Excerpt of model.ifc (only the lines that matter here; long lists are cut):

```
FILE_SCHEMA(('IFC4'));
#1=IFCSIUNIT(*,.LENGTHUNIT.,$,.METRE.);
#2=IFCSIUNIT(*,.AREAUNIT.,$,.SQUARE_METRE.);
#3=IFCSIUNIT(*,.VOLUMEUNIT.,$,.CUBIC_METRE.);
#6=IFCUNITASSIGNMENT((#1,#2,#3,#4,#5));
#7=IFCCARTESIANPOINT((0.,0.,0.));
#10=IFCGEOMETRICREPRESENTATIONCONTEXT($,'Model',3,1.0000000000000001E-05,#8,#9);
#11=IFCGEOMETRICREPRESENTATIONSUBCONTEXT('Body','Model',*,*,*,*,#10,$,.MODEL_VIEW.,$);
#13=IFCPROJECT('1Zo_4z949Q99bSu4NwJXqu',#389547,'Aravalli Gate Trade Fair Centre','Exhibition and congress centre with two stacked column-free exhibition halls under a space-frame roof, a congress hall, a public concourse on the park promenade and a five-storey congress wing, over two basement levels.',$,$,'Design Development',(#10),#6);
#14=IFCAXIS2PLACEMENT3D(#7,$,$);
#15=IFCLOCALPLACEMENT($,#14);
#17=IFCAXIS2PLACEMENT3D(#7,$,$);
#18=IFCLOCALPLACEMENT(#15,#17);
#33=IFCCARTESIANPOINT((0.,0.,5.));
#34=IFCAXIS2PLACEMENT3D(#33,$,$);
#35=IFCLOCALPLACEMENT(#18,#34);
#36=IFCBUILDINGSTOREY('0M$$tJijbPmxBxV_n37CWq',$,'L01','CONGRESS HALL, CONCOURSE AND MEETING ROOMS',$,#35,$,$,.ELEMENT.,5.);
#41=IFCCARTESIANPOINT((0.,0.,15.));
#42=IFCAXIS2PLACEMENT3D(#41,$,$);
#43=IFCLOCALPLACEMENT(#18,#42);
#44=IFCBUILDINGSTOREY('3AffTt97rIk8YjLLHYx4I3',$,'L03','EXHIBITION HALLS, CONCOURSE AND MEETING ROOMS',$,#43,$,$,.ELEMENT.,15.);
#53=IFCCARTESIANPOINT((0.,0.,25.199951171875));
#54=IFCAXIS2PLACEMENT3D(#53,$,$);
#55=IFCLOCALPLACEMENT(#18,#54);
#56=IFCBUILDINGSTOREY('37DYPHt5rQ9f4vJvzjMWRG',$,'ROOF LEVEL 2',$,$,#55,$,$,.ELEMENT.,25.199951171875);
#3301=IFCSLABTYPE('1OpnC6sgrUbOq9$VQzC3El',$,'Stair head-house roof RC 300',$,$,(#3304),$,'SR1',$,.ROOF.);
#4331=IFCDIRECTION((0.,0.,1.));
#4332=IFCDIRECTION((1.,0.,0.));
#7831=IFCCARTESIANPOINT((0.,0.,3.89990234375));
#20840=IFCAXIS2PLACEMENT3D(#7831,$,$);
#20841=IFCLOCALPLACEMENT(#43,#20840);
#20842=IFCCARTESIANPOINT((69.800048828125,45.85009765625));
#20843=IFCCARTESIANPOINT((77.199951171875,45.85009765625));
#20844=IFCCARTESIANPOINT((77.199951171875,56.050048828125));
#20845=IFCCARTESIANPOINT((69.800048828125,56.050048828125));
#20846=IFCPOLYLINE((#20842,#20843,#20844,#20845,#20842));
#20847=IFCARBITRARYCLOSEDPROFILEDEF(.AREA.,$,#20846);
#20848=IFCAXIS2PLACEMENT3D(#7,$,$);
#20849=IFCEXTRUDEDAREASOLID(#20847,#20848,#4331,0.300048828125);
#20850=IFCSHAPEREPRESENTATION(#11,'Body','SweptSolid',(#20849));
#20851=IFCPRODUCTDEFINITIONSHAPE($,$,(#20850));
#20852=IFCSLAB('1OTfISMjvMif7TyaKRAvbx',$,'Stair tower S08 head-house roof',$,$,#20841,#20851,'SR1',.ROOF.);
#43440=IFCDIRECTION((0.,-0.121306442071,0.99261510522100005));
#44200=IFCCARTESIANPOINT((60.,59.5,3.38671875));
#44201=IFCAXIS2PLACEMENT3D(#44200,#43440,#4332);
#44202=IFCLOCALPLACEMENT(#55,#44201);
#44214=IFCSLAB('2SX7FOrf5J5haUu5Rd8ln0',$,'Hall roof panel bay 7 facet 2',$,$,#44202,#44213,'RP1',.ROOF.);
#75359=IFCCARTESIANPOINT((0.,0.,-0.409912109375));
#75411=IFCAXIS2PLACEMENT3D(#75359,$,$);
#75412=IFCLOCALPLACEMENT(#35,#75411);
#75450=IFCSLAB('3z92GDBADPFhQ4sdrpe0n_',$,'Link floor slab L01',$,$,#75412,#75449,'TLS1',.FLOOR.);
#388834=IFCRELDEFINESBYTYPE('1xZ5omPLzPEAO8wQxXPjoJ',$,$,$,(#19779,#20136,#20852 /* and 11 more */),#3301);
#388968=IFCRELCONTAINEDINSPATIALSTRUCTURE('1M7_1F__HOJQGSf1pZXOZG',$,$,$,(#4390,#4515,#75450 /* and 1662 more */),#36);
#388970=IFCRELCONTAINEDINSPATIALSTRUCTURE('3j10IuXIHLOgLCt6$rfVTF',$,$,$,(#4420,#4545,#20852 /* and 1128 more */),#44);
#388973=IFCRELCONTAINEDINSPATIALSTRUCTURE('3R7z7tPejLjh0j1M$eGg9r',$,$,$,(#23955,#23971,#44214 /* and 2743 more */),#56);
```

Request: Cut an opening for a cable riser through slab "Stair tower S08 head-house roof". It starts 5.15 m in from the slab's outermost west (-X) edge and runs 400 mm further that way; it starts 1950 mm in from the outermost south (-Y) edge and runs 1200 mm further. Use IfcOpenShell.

```python
import numpy as np
import ifcopenshell
import ifcopenshell.api.feature
import ifcopenshell.api.geometry
import ifcopenshell.api.root
import ifcopenshell.geom
import ifcopenshell.util.placement
import ifcopenshell.util.representation
import ifcopenshell.util.shape
import ifcopenshell.util.unit

model = ifcopenshell.open("model.ifc")
unit_scale = ifcopenshell.util.unit.calculate_unit_scale(model)
settings = ifcopenshell.geom.settings()


def volume(element):
    """Net volume in cubic metres, openings subtracted."""
    shape = ifcopenshell.geom.create_shape(settings, element)
    return ifcopenshell.util.shape.get_volume(shape.geometry)


slab = model.by_guid("1OTfISMjvMif7TyaKRAvbx")
before = volume(slab)

# Extent in the slab's own axes, in metres. The edges named are its -X and -Y sides.
slab_shape = ifcopenshell.geom.create_shape(settings, slab)
vertices = ifcopenshell.util.shape.get_vertices(slab_shape.geometry)
x_min, y_min, bottom = vertices.min(axis=0)
top = vertices[:, 2].max()

opening = ifcopenshell.api.root.create_entity(model, ifc_class="IfcOpeningElement", name="Cable riser opening", predefined_type="OPENING")
context = ifcopenshell.util.representation.get_context(model, "Model", "Body", "MODEL_VIEW")
width, depth = 0.4, 1.2
outline = [(0.0, 0.0), (width, 0.0), (width, depth), (0.0, depth), (0.0, 0.0)]
# Overshoot both faces by 50 mm so the cut is clean.
shape = ifcopenshell.api.geometry.add_slab_representation(
    model, context=context, depth=top - bottom + 0.1, polyline=outline
)
ifcopenshell.api.geometry.assign_representation(model, product=opening, representation=shape)

matrix = ifcopenshell.util.placement.get_local_placement(slab.ObjectPlacement)
matrix[:, 3] = matrix @ np.append(np.array([x_min + 5.15, y_min + 1.95, bottom - 0.05]) / unit_scale, 1.0)
ifcopenshell.api.geometry.edit_object_placement(model, product=opening, matrix=matrix, is_si=False)
ifcopenshell.api.feature.add_feature(model, feature=opening, element=slab)

after = volume(slab)

print(f"slab volume {before:.3f} -> {after:.3f} m3")

model.write("model_updated.ifc")
```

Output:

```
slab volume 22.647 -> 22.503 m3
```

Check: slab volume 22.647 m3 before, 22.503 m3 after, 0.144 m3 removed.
